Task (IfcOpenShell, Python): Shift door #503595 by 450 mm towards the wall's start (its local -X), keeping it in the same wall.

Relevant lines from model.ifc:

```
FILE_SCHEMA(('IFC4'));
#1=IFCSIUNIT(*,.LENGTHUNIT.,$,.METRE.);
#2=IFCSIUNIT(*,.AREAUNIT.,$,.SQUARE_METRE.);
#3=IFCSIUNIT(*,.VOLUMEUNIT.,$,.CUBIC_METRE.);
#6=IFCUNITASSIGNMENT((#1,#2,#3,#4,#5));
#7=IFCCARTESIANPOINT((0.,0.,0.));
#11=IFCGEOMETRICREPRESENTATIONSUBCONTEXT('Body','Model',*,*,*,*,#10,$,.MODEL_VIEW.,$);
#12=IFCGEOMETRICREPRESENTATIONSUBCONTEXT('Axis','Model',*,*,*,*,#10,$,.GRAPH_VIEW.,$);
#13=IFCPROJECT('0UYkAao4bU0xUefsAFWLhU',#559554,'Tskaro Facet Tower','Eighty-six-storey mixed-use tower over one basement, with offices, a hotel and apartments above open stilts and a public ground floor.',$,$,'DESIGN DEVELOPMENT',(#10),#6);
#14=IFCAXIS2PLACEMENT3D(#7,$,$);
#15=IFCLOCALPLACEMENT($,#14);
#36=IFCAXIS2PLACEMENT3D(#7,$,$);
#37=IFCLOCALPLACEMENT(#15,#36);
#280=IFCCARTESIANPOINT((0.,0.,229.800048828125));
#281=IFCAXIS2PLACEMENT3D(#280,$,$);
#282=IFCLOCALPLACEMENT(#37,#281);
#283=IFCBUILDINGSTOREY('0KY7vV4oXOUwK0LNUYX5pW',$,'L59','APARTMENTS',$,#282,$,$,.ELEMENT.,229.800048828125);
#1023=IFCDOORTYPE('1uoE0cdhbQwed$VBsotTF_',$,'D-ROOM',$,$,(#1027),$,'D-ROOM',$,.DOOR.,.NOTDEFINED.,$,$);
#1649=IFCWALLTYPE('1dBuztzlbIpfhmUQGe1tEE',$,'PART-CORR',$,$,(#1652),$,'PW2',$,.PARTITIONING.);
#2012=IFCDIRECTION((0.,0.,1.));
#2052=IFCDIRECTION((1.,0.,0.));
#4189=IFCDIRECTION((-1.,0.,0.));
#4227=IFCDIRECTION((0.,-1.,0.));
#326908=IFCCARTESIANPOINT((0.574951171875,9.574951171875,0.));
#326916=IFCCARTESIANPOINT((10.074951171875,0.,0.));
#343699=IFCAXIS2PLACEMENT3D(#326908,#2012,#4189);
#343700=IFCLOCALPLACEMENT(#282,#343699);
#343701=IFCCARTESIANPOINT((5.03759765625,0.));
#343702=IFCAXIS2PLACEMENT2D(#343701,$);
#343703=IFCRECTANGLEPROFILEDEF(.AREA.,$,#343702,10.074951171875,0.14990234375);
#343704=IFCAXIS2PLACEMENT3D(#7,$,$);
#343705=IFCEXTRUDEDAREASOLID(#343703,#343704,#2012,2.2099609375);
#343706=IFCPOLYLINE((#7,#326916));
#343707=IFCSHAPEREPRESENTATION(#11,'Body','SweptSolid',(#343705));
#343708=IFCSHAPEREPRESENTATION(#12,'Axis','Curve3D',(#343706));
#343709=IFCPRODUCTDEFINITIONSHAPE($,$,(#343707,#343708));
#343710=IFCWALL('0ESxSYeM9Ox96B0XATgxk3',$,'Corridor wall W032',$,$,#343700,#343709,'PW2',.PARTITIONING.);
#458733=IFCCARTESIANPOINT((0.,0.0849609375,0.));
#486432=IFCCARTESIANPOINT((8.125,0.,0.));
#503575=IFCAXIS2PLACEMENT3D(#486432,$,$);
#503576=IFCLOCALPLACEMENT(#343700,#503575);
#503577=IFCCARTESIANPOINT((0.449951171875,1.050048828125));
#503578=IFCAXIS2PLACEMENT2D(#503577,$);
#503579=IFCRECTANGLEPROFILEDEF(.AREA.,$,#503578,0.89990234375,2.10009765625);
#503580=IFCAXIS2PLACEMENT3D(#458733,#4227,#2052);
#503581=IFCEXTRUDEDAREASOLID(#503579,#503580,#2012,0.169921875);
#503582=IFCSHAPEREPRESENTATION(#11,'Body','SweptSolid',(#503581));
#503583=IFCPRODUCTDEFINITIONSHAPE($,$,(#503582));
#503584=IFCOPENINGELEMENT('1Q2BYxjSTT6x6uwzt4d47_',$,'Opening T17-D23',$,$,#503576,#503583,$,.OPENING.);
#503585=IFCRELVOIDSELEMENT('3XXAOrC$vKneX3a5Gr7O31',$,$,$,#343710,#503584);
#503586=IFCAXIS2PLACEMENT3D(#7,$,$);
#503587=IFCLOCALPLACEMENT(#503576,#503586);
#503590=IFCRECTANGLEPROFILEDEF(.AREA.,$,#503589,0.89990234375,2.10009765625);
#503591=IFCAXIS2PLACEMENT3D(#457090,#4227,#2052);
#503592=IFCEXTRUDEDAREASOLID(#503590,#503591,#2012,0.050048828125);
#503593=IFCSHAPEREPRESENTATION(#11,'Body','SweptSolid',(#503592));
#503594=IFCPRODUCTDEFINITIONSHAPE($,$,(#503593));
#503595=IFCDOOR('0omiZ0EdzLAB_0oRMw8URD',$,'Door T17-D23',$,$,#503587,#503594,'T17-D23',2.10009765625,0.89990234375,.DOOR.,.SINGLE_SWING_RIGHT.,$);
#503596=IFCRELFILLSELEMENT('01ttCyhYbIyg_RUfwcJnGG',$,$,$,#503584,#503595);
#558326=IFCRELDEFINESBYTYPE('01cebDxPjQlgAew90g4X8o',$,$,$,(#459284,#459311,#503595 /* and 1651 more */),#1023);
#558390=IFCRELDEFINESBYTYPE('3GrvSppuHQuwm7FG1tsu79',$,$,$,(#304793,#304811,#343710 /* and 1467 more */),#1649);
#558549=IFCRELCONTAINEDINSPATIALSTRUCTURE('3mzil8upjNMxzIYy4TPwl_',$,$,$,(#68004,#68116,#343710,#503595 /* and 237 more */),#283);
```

```python
import ifcopenshell
import ifcopenshell.api.geometry
import ifcopenshell.util.placement
import ifcopenshell.util.unit

model = ifcopenshell.open("model.ifc")
unit_scale = ifcopenshell.util.unit.calculate_unit_scale(model)

door = model.by_id(503595)
opening = door.FillsVoids[0].RelatingOpeningElement
wall = opening.VoidsElements[0].RelatingBuildingElement

wall_matrix = ifcopenshell.util.placement.get_local_placement(wall.ObjectPlacement)
shift = wall_matrix[:3, 0] * -0.45 / unit_scale
before = ifcopenshell.util.placement.get_local_placement(door.ObjectPlacement)[:3, 3].copy()

# The door is placed relative to its opening, so it follows when the opening moves.
matrix = ifcopenshell.util.placement.get_local_placement(opening.ObjectPlacement)
matrix[:3, 3] += shift
ifcopenshell.api.geometry.edit_object_placement(
    model, product=opening, matrix=matrix, is_si=False, should_transform_children=True
)

after = ifcopenshell.util.placement.get_local_placement(door.ObjectPlacement)[:3, 3]
print("door moved by", (after - before).round(3) + 0.0)

model.write("model_edited.ifc")
```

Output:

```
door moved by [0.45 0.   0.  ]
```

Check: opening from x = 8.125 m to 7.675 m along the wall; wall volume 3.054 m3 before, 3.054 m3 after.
